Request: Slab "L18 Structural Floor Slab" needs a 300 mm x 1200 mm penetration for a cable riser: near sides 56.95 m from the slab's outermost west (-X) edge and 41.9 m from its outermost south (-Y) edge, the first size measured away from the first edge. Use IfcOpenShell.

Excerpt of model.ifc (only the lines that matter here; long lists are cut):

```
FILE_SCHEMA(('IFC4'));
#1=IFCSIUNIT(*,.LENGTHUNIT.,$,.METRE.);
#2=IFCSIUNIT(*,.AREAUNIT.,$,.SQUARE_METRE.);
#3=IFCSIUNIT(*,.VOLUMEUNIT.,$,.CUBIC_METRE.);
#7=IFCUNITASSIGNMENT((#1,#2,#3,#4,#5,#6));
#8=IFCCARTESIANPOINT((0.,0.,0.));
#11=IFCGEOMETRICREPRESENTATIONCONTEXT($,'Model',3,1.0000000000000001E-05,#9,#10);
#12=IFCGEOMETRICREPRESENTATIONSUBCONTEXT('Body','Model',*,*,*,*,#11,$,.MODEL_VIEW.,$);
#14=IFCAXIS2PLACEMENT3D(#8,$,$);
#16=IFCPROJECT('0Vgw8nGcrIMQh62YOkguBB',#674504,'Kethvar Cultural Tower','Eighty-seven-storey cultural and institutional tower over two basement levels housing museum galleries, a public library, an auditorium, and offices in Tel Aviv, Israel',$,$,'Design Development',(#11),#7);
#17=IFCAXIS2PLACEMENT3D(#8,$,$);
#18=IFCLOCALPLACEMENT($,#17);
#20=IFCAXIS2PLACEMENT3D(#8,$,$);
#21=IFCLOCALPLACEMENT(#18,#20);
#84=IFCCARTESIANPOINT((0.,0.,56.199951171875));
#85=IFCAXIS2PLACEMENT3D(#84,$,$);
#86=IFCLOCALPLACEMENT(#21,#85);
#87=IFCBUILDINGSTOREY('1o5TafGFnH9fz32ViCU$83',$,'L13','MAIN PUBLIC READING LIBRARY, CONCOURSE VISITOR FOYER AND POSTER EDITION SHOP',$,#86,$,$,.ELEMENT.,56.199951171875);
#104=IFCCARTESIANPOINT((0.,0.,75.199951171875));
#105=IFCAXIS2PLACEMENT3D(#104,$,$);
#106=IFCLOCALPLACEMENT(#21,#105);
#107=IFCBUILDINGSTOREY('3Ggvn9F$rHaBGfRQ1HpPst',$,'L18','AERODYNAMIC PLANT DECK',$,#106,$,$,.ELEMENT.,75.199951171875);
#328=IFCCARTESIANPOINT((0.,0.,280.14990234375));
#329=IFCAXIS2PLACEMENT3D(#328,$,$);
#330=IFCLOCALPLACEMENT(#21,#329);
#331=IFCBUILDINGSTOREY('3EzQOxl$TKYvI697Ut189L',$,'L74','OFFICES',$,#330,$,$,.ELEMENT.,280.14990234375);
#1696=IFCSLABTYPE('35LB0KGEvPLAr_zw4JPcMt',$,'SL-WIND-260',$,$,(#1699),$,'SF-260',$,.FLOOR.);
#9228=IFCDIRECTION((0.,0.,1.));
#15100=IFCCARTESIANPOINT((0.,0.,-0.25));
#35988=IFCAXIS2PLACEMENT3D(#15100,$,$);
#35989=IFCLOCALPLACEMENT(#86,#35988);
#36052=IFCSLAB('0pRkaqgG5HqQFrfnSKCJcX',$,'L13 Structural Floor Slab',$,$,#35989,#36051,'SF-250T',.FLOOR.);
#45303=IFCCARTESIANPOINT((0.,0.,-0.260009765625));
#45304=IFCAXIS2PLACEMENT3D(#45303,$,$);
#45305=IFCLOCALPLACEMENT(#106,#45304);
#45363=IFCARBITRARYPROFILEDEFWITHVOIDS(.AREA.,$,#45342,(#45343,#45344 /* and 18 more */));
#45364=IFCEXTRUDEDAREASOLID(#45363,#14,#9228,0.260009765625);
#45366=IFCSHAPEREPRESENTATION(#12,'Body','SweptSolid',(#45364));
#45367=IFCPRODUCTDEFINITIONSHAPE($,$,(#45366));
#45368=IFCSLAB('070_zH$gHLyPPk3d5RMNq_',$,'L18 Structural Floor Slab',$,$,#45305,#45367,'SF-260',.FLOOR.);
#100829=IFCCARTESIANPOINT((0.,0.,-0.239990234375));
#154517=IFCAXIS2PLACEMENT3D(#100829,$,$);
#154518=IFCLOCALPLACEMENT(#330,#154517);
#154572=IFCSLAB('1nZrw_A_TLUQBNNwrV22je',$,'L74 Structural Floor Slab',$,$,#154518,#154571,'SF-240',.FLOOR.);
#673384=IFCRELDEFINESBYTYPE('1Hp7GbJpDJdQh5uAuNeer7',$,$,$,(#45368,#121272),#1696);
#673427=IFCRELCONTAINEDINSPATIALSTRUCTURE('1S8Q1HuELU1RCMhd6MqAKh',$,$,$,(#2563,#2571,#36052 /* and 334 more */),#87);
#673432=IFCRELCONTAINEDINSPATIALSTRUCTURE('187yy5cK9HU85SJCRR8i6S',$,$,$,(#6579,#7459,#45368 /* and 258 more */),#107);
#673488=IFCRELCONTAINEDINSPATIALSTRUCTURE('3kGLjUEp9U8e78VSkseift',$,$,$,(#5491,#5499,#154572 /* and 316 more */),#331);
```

```python
import numpy as np
import ifcopenshell
import ifcopenshell.api.feature
import ifcopenshell.api.geometry
import ifcopenshell.api.root
import ifcopenshell.geom
import ifcopenshell.util.placement
import ifcopenshell.util.representation
import ifcopenshell.util.shape
import ifcopenshell.util.unit

model = ifcopenshell.open("model.ifc")
unit_scale = ifcopenshell.util.unit.calculate_unit_scale(model)
settings = ifcopenshell.geom.settings()


def volume(element):
    """Net volume in cubic metres, openings subtracted."""
    shape = ifcopenshell.geom.create_shape(settings, element)
    return ifcopenshell.util.shape.get_volume(shape.geometry)


slab = model.by_guid("070_zH$gHLyPPk3d5RMNq_")
before = volume(slab)

# Extent in the slab's own axes, in metres. The edges named are its -X and -Y sides.
slab_shape = ifcopenshell.geom.create_shape(settings, slab)
vertices = ifcopenshell.util.shape.get_vertices(slab_shape.geometry)
x_min, y_min, bottom = vertices.min(axis=0)
top = vertices[:, 2].max()

opening = ifcopenshell.api.root.create_entity(model, ifc_class="IfcOpeningElement", name="Cable riser opening", predefined_type="OPENING")
context = ifcopenshell.util.representation.get_context(model, "Model", "Body", "MODEL_VIEW")
width, depth = 0.3, 1.2
outline = [(0.0, 0.0), (width, 0.0), (width, depth), (0.0, depth), (0.0, 0.0)]
# Overshoot both faces by 50 mm so the cut is clean.
shape = ifcopenshell.api.geometry.add_slab_representation(
    model, context=context, depth=top - bottom + 0.1, polyline=outline
)
ifcopenshell.api.geometry.assign_representation(model, product=opening, representation=shape)

matrix = ifcopenshell.util.placement.get_local_placement(slab.ObjectPlacement)
matrix[:, 3] = matrix @ np.append(np.array([x_min + 56.95, y_min + 41.9, bottom - 0.05]) / unit_scale, 1.0)
ifcopenshell.api.geometry.edit_object_placement(model, product=opening, matrix=matrix, is_si=False)
ifcopenshell.api.feature.add_feature(model, feature=opening, element=slab)

after = volume(slab)

print(f"slab volume {before:.3f} -> {after:.3f} m3")

model.write("model_rev.ifc")
```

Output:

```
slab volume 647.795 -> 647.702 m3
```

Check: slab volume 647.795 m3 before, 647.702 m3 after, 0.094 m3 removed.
